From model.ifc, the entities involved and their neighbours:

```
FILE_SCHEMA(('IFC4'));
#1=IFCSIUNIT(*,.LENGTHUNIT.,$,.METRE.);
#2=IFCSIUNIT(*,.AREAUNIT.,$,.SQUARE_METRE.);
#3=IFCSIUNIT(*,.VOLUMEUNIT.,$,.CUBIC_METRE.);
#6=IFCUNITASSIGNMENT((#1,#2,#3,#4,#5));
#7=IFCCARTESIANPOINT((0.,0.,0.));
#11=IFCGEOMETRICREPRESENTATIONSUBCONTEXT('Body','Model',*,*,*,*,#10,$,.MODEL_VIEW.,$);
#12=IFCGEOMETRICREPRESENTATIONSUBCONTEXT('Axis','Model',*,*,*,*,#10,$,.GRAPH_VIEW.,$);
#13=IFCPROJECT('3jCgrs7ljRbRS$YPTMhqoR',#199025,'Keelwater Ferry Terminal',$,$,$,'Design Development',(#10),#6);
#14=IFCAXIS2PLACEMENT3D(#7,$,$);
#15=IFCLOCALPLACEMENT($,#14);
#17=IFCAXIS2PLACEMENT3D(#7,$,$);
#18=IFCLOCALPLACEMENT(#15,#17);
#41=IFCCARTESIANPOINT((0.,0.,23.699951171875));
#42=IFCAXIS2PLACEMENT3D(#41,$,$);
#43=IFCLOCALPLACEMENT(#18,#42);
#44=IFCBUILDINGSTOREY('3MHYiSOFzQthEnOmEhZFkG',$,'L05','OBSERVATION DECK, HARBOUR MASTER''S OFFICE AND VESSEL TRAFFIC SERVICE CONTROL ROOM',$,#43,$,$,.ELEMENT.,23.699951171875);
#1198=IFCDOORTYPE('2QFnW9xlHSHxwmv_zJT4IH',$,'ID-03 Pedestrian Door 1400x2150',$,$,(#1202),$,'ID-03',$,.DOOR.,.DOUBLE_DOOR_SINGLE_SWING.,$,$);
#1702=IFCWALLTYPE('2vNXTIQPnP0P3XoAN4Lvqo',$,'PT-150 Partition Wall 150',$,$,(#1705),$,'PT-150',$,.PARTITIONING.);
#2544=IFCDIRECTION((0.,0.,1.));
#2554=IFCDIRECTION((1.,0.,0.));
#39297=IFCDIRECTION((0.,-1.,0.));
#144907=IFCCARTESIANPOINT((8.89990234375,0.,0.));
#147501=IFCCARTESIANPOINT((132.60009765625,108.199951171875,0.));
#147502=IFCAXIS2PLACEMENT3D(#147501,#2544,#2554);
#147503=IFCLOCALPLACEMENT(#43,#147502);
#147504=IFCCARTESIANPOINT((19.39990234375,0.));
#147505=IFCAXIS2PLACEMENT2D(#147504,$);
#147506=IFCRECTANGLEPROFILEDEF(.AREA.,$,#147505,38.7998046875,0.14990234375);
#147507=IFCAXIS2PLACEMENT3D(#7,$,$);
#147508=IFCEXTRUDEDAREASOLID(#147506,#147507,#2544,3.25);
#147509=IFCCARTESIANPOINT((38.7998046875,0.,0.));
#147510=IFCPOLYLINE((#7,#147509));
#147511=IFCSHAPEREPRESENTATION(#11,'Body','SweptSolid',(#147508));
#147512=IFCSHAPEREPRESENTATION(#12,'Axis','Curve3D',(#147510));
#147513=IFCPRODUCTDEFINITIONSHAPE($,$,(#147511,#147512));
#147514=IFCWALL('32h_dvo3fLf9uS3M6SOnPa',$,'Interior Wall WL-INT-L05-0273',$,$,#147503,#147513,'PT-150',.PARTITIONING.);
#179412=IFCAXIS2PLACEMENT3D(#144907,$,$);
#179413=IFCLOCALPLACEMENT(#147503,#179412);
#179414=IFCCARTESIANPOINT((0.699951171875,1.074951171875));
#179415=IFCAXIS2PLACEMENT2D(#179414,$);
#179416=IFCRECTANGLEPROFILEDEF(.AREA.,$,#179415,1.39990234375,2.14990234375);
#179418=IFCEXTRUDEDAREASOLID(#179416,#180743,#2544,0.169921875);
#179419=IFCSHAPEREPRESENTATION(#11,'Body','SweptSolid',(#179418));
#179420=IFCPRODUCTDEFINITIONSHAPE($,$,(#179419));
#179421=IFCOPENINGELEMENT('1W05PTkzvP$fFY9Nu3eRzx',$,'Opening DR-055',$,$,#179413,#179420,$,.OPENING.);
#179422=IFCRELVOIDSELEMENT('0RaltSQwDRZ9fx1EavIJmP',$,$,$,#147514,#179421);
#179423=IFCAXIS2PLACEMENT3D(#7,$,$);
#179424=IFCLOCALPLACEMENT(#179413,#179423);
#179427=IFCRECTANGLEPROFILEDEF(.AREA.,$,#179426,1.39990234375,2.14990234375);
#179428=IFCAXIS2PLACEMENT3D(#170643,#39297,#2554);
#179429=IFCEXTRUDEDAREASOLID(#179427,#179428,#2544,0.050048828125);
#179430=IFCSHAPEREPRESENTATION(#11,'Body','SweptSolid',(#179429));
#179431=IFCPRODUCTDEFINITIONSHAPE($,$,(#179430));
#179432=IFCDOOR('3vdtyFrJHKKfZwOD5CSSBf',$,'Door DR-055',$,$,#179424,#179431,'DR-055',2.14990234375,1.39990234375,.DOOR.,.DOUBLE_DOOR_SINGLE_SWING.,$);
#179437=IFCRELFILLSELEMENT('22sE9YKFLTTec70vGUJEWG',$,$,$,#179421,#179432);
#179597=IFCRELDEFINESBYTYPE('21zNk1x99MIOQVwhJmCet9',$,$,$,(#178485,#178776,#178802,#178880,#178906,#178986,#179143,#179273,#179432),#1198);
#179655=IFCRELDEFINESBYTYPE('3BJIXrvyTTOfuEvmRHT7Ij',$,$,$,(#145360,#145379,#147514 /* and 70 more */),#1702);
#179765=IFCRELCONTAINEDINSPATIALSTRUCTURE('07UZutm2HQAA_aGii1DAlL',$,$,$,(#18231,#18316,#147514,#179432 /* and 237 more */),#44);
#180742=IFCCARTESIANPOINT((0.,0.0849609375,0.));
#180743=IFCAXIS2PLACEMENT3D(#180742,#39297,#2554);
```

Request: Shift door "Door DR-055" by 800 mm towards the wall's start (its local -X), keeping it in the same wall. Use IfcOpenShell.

```python
import ifcopenshell
import ifcopenshell.api.geometry
import ifcopenshell.util.placement

model = ifcopenshell.open("model.ifc")

door = model.by_guid("3vdtyFrJHKKfZwOD5CSSBf")
opening = door.FillsVoids[0].RelatingOpeningElement
wall = opening.VoidsElements[0].RelatingBuildingElement

wall_matrix = ifcopenshell.util.placement.get_local_placement(wall.ObjectPlacement)
shift = wall_matrix[:3, 0] * -0.8
before = ifcopenshell.util.placement.get_local_placement(door.ObjectPlacement)[:3, 3].copy()

# The door is placed relative to its opening, so it follows when the opening moves.
matrix = ifcopenshell.util.placement.get_local_placement(opening.ObjectPlacement)
matrix[:3, 3] += shift
ifcopenshell.api.geometry.edit_object_placement(
    model, product=opening, matrix=matrix, is_si=False, should_transform_children=True
)

after = ifcopenshell.util.placement.get_local_placement(door.ObjectPlacement)[:3, 3]
print("door moved by", (after - before).round(3) + 0.0)

model.write("model-out.ifc")
```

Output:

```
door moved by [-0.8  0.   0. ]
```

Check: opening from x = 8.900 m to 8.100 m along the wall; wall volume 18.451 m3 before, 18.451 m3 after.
